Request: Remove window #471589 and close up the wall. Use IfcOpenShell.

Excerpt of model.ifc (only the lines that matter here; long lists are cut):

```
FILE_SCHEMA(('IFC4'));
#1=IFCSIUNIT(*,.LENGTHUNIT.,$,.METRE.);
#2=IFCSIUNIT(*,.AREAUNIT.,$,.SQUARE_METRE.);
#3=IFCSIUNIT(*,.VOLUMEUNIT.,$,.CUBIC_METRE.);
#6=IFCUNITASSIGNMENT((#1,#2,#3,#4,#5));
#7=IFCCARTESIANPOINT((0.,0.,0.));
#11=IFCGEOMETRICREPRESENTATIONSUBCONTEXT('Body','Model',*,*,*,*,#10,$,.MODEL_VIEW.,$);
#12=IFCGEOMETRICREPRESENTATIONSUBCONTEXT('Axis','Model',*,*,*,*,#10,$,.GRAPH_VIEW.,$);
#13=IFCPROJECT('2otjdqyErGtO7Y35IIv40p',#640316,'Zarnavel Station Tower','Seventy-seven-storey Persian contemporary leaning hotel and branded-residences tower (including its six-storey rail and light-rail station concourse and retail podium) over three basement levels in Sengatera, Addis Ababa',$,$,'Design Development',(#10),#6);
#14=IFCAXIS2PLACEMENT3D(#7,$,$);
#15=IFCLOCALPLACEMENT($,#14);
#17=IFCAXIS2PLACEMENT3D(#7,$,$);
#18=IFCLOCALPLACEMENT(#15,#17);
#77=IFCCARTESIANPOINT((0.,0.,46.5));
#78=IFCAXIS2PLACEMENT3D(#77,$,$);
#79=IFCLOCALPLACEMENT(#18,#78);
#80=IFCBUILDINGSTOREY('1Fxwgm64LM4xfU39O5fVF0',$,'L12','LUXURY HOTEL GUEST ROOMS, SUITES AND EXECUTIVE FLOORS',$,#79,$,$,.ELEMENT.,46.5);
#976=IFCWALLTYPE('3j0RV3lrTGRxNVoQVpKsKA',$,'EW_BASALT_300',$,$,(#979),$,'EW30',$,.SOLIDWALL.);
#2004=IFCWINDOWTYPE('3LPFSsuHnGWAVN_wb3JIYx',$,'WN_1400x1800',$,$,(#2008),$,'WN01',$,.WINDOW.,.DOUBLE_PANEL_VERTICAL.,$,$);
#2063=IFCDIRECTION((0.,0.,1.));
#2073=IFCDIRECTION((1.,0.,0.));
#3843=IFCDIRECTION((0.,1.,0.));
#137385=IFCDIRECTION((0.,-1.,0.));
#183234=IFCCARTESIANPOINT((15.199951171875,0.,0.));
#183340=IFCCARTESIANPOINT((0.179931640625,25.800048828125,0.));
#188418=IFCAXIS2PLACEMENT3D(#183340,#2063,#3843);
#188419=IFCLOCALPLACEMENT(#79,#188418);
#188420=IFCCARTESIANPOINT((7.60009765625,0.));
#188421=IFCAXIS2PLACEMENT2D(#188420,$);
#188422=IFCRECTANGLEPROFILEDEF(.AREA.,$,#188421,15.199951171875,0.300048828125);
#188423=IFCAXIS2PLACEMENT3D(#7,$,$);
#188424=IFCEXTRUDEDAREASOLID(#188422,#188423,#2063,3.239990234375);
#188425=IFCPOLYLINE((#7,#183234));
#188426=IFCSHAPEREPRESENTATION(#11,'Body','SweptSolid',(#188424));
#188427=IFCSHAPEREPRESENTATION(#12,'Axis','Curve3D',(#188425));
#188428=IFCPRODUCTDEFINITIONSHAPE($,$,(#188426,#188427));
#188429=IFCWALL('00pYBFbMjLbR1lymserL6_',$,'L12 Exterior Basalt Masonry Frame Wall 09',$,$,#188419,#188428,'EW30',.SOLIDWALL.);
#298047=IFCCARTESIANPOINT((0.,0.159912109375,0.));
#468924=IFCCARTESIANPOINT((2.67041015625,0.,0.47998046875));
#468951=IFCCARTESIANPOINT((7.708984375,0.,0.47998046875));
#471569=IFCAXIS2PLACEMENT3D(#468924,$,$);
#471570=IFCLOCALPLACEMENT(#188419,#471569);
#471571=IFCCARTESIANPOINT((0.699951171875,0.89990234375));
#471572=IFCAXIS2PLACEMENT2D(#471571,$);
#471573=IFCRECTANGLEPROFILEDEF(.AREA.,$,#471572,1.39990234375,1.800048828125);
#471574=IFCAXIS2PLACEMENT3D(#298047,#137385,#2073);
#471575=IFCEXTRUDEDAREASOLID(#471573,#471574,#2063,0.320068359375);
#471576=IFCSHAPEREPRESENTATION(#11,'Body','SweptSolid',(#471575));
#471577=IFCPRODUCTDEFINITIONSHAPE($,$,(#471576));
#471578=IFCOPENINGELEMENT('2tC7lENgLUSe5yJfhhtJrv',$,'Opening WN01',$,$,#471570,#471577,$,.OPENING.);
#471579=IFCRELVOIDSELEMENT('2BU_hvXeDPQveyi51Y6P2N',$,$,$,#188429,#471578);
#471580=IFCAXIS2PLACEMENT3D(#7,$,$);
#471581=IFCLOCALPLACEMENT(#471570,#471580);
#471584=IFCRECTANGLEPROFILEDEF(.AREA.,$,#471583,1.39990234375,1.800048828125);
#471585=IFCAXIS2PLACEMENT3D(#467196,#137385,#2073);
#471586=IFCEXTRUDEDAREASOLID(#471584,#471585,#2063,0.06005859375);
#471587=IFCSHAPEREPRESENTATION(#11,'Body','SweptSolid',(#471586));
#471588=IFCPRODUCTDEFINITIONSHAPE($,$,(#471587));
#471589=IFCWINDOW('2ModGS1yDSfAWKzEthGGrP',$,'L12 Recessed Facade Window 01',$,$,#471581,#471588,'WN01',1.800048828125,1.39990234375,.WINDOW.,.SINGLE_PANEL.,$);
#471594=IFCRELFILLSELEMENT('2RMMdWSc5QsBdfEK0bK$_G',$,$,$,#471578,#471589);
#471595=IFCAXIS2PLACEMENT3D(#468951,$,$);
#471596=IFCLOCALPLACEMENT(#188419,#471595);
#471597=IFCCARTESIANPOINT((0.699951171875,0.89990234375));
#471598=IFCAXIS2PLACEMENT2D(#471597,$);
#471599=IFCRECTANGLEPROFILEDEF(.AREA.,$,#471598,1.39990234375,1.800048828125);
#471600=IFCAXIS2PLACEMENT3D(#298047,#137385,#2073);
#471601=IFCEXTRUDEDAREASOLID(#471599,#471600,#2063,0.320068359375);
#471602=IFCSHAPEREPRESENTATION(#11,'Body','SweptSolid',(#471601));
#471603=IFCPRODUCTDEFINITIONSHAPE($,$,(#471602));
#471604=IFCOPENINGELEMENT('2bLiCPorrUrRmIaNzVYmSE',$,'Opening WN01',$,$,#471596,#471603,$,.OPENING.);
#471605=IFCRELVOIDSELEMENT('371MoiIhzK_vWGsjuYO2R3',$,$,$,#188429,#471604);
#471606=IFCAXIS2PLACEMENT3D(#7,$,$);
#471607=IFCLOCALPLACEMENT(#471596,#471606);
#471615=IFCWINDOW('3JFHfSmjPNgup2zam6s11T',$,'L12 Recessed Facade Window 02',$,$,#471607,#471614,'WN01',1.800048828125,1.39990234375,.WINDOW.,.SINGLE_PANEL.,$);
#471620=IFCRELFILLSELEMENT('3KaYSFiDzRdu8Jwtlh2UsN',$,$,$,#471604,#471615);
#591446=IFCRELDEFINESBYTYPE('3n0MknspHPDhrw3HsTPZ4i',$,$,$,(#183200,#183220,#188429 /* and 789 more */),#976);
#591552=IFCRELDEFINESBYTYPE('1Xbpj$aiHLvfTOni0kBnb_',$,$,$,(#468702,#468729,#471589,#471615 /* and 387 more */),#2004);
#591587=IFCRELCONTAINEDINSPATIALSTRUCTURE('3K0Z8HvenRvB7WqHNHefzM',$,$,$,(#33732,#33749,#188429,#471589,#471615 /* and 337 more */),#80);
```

```python
import ifcopenshell
import ifcopenshell.api.feature
import ifcopenshell.api.root
import ifcopenshell.geom
import ifcopenshell.util.shape

model = ifcopenshell.open("model.ifc")
settings = ifcopenshell.geom.settings()


def volume(element):
    """Net volume in cubic metres, openings subtracted."""
    shape = ifcopenshell.geom.create_shape(settings, element)
    return ifcopenshell.util.shape.get_volume(shape.geometry)


window = model.by_guid("2ModGS1yDSfAWKzEthGGrP")
opening = window.FillsVoids[0].RelatingOpeningElement
wall = opening.VoidsElements[0].RelatingBuildingElement
before = volume(wall)

ifcopenshell.api.root.remove_product(model, product=window)
ifcopenshell.api.feature.remove_feature(model, feature=opening)

after = volume(wall)

print(f"wall volume {before:.3f} -> {after:.3f} m3")

model.write("model_rev.ifc")
```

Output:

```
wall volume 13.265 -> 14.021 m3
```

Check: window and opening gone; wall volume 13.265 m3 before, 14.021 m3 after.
